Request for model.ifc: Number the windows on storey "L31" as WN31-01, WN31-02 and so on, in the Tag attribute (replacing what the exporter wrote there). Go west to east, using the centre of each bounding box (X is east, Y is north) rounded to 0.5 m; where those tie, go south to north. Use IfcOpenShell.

First a look at what the model holds.

```python
import ifcopenshell
import ifcopenshell.util.element
import ifcopenshell.util.placement

model = ifcopenshell.open("model.ifc")
print(model.schema)
storey = next(s for s in model.by_type("IfcBuildingStorey") if s.Name == "L31")
windows = [e for e in ifcopenshell.util.element.get_decomposition(storey) if e.is_a("IfcWindow")]
for e in sorted(windows, key=lambda e: e.id()):
    origin = ifcopenshell.util.placement.get_local_placement(e.ObjectPlacement)[:3, 3]
    print(e.id(), e.Tag, e.Name, origin.round(2) + 0.0, sep=" | ")
```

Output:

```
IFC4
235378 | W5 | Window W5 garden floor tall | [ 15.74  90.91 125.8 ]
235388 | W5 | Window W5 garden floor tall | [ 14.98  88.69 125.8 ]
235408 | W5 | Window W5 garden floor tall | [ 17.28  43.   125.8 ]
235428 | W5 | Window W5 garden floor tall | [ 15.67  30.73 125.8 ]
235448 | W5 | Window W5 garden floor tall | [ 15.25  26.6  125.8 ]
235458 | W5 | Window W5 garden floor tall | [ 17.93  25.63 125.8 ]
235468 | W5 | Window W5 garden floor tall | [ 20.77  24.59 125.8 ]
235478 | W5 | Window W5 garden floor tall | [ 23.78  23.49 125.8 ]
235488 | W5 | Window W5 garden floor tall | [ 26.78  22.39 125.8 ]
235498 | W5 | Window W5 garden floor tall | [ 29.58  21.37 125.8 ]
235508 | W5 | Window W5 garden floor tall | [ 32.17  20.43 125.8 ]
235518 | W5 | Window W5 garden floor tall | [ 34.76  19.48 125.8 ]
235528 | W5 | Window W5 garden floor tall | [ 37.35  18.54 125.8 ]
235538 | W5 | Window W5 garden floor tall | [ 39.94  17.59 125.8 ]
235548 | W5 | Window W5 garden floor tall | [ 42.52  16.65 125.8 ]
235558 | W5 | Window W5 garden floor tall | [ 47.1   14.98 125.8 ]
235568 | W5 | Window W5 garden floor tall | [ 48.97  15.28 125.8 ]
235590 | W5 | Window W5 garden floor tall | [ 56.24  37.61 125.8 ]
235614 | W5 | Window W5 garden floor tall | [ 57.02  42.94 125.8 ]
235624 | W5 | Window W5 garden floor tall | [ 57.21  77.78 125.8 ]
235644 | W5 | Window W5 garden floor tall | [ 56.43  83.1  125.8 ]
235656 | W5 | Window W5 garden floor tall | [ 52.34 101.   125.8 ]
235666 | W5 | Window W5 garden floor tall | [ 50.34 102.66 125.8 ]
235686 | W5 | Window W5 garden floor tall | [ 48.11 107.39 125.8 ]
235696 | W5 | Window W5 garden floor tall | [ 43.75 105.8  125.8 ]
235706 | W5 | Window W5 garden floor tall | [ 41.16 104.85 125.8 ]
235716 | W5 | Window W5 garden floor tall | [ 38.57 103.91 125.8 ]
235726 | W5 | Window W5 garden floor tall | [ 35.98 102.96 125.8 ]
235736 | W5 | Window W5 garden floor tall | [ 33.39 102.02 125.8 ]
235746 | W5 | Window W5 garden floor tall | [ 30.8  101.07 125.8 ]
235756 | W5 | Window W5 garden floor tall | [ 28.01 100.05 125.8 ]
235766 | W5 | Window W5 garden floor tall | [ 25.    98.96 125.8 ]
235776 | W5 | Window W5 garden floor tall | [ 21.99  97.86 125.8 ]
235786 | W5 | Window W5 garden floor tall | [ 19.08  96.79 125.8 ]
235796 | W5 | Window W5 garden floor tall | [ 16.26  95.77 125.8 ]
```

```python
import ifcopenshell
import ifcopenshell.geom
import ifcopenshell.util.element
import ifcopenshell.util.shape

model = ifcopenshell.open("model.ifc")
settings = ifcopenshell.geom.settings()
settings.set("use-world-coords", True)


def centre(element):
    shape = ifcopenshell.geom.create_shape(settings, element)
    return ifcopenshell.util.shape.get_bbox_centroid(shape.geometry)


storey = next(s for s in model.by_type("IfcBuildingStorey") if s.Name == "L31")
windows = [e for e in ifcopenshell.util.element.get_decomposition(storey) if e.is_a("IfcWindow")]

# Insertion points can sit at a corner or the storey origin, so sort by the geometry (in metres).
centres = {e: centre(e) for e in windows}
windows.sort(key=lambda e: (round(centres[e][0] / 0.5), centres[e][1]))

for i, e in enumerate(windows, start=1):
    number = f"WN31-{i:02d}"
    e.Tag = number
    print(e.id(), number)

model.write("model_v2.ifc")
```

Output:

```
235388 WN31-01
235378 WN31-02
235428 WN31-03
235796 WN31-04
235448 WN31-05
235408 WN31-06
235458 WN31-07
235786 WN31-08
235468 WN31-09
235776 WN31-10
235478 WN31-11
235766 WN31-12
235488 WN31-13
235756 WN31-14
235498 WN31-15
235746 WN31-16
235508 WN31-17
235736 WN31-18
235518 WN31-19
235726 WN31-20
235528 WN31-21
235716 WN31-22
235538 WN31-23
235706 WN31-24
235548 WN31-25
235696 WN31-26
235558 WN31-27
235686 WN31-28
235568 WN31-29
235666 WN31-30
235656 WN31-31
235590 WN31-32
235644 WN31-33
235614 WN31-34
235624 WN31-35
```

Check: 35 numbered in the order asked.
